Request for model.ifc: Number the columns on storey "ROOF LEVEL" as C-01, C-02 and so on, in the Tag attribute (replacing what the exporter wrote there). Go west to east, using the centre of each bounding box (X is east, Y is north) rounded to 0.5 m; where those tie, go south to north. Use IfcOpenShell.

First a look at what the model holds.

```python
import ifcopenshell
import ifcopenshell.util.element
import ifcopenshell.util.placement

model = ifcopenshell.open("model.ifc")
print(model.schema)
storey = next(s for s in model.by_type("IfcBuildingStorey") if s.Name == "ROOF LEVEL")
columns = [e for e in ifcopenshell.util.element.get_decomposition(storey) if e.is_a("IfcColumn")]
for e in sorted(columns, key=lambda e: e.id()):
    origin = ifcopenshell.util.placement.get_local_placement(e.ObjectPlacement)[:3, 3]
    print(e.id(), e.Tag, e.Name, origin.round(2) + 0.0, sep=" | ")
```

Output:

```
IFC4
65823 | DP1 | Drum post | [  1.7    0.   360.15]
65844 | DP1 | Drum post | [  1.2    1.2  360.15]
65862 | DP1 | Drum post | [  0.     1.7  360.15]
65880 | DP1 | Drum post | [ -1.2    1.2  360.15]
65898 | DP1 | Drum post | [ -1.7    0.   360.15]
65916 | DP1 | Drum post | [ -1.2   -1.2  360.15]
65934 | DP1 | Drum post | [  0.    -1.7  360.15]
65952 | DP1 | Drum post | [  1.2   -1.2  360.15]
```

```python
import ifcopenshell
import ifcopenshell.geom
import ifcopenshell.util.element
import ifcopenshell.util.shape

model = ifcopenshell.open("model.ifc")
settings = ifcopenshell.geom.settings()
settings.set("use-world-coords", True)


def centre(element):
    shape = ifcopenshell.geom.create_shape(settings, element)
    return ifcopenshell.util.shape.get_bbox_centroid(shape.geometry)


storey = next(s for s in model.by_type("IfcBuildingStorey") if s.Name == "ROOF LEVEL")
columns = [e for e in ifcopenshell.util.element.get_decomposition(storey) if e.is_a("IfcColumn")]

# Insertion points can sit at a corner or the storey origin, so sort by the geometry (in metres).
centres = {e: centre(e) for e in columns}
columns.sort(key=lambda e: (round(centres[e][0] / 0.5), centres[e][1]))

for i, e in enumerate(columns, start=1):
    number = f"C-{i:02d}"
    e.Tag = number
    print(e.id(), number)

model.write("model-out.ifc")
```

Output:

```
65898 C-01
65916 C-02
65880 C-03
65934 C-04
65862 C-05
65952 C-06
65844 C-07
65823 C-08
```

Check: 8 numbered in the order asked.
